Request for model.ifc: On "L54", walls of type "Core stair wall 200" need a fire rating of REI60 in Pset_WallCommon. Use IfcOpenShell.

First a look at what the model holds.

```python
import ifcopenshell
import ifcopenshell.util.element

model = ifcopenshell.open("model.ifc")
print(model.schema)
storey = next(s for s in model.by_type("IfcBuildingStorey") if s.Name == "L54")
walls = [e for e in ifcopenshell.util.element.get_decomposition(storey) if e.is_a("IfcWall")]
seen = {}
for e in walls:
    element_type = ifcopenshell.util.element.get_type(e)
    key = (element_type.Name if element_type != e and element_type else None, ifcopenshell.util.element.get_pset(e, "Pset_WallCommon", "FireRating"))
    seen[key] = seen.get(key, 0) + 1
for (name, value), count in sorted(seen.items(), key=str):
    print(count, "x", name, "|", value)
```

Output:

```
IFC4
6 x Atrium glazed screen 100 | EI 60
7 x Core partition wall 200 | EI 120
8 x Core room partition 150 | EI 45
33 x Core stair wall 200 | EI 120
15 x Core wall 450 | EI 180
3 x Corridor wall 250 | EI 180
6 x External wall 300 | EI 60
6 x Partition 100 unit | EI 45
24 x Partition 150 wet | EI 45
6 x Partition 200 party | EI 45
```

```python
import ifcopenshell
import ifcopenshell.api.pset
import ifcopenshell.util.element

model = ifcopenshell.open("model.ifc")

storey = next(s for s in model.by_type("IfcBuildingStorey") if s.Name == "L54")
walls = [e for e in ifcopenshell.util.element.get_decomposition(storey) if e.is_a("IfcWall")]

count = 0
for e in walls:
    element_type = ifcopenshell.util.element.get_type(e)
    if element_type in (None, e) or element_type.Name != "Core stair wall 200":
        continue
    found = ifcopenshell.util.element.get_pset(e, "Pset_WallCommon", should_inherit=False)
    if found:
        pset = model.by_id(found["id"])
        if len(ifcopenshell.util.element.get_elements_by_pset(pset)) > 1:
            pset = ifcopenshell.api.pset.unshare_pset(model, products=[e], pset=pset)[0]
    else:
        pset = ifcopenshell.api.pset.add_pset(model, product=e, name="Pset_WallCommon")
    ifcopenshell.api.pset.edit_pset(model, pset=pset, properties={"FireRating": "REI60"})
    count += 1

print(count, "walls updated")

model.write("model_rev.ifc")
```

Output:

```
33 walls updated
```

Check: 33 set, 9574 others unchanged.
